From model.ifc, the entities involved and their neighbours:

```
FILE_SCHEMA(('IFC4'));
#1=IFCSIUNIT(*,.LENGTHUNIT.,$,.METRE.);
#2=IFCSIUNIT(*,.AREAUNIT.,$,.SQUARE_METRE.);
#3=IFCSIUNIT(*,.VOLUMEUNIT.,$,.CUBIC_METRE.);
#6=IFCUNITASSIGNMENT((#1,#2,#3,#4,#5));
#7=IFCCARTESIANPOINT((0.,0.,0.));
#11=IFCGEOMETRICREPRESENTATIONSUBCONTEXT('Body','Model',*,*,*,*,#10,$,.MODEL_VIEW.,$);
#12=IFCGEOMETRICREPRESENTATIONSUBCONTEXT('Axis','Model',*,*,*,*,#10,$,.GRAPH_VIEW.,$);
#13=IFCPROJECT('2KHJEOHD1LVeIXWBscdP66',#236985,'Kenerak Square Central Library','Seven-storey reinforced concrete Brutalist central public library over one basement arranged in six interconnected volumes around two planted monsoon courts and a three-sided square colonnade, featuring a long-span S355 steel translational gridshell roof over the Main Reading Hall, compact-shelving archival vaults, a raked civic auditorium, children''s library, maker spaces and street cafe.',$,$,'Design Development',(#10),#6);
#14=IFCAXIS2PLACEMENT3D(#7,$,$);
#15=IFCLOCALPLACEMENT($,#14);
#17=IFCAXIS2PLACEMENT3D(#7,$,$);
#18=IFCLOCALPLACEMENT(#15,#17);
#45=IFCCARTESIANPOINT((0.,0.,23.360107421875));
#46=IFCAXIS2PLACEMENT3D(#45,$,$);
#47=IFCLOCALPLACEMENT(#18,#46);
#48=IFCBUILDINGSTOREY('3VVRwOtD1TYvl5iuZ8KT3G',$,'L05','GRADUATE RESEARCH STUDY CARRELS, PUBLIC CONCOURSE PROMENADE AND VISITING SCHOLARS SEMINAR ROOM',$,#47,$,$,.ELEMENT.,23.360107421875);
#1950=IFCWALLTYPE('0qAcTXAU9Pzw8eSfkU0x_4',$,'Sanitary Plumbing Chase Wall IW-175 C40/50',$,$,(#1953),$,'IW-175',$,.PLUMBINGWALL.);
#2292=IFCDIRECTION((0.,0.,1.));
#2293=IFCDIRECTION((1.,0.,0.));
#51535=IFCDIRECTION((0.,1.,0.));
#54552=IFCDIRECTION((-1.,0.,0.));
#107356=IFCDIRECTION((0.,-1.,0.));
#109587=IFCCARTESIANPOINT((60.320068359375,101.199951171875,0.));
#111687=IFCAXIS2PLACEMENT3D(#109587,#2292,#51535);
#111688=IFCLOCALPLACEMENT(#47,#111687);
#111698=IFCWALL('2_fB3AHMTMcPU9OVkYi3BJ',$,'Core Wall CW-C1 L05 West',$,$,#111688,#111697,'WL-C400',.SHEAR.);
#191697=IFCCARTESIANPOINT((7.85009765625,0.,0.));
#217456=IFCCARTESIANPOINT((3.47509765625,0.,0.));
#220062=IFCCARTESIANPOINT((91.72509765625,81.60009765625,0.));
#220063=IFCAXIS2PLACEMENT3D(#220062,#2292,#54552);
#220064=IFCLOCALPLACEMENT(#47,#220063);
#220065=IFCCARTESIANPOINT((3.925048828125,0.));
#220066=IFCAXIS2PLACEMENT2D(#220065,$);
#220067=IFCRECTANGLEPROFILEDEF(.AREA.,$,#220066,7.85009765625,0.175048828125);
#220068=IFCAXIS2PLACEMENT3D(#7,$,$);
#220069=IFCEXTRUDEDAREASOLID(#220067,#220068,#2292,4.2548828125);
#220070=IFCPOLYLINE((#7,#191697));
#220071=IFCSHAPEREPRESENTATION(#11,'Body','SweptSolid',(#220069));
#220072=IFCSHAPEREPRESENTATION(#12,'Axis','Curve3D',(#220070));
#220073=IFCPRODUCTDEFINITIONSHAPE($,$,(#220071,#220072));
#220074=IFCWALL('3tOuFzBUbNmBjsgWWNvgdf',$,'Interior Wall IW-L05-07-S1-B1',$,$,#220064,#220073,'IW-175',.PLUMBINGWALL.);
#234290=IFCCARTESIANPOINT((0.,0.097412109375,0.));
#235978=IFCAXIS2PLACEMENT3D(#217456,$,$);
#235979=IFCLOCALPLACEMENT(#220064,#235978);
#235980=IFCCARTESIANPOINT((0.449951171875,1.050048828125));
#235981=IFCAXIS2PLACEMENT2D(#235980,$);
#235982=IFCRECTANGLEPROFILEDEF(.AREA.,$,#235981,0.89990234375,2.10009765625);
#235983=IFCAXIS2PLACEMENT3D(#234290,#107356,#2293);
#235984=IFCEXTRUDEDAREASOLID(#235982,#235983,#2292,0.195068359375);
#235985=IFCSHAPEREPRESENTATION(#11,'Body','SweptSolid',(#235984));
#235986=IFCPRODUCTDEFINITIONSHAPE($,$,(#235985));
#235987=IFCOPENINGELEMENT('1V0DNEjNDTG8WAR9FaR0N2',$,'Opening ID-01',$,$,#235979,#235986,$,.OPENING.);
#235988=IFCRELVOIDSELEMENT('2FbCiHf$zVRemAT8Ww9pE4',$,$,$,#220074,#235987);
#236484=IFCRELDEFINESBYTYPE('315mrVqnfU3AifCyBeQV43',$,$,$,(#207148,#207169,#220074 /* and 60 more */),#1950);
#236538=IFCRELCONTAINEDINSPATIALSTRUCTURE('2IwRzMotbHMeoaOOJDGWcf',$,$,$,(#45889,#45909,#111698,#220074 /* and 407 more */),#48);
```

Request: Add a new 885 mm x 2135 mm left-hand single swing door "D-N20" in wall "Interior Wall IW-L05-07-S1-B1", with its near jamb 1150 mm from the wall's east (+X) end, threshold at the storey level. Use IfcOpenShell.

```python
import numpy as np
import ifcopenshell
import ifcopenshell.api.feature
import ifcopenshell.api.geometry
import ifcopenshell.api.root
import ifcopenshell.api.spatial
import ifcopenshell.geom
import ifcopenshell.util.element
import ifcopenshell.util.placement
import ifcopenshell.util.representation
import ifcopenshell.util.shape
import ifcopenshell.util.unit

model = ifcopenshell.open("model.ifc")
unit_scale = ifcopenshell.util.unit.calculate_unit_scale(model)
settings = ifcopenshell.geom.settings()


def volume(element):
    """Net volume in cubic metres, openings subtracted."""
    shape = ifcopenshell.geom.create_shape(settings, element)
    return ifcopenshell.util.shape.get_volume(shape.geometry)


wall = model.by_guid("3tOuFzBUbNmBjsgWWNvgdf")
storey = ifcopenshell.util.element.get_container(wall, ifc_class="IfcBuildingStorey")
context = ifcopenshell.util.representation.get_context(model, "Model", "Body", "MODEL_VIEW")
before = volume(wall)

width, height, from_end, sill = 0.885, 2.135, 1.15, 0.0  # metres

# The wall runs along its own X axis, and the end named is its -X end.
wall_shape = ifcopenshell.geom.create_shape(settings, wall)
x, y, z = ifcopenshell.util.shape.get_vertices(wall_shape.geometry).T
start = x.min() + from_end
face, thickness = float(y.min()), float(y.max() - y.min())
wall_matrix = ifcopenshell.util.placement.get_local_placement(wall.ObjectPlacement)
level = ifcopenshell.util.placement.get_local_placement(storey.ObjectPlacement)[2, 3]


def in_wall(x, y):
    """Placement at x, y metres in the wall's axes, at sill height."""
    matrix = wall_matrix.copy()
    matrix[:, 3] = wall_matrix @ np.array([x / unit_scale, y / unit_scale, 0.0, 1.0])
    matrix[2, 3] = level + sill / unit_scale
    return matrix


# Opening: a box that overshoots both wall faces by 50 mm.
opening = ifcopenshell.api.root.create_entity(model, ifc_class="IfcOpeningElement", predefined_type="OPENING")
box = ifcopenshell.api.geometry.add_wall_representation(
    model, context=context, length=width, height=height, thickness=thickness + 0.1
)
ifcopenshell.api.geometry.assign_representation(model, product=opening, representation=box)
ifcopenshell.api.geometry.edit_object_placement(model, product=opening, matrix=in_wall(start, face - 0.05), is_si=False)
ifcopenshell.api.feature.add_feature(model, feature=opening, element=wall)

door = ifcopenshell.api.root.create_entity(model, ifc_class="IfcDoor", name="D-N20", predefined_type="DOOR")
door.OverallWidth, door.OverallHeight = width / unit_scale, height / unit_scale
door.OperationType = "SINGLE_SWING_LEFT"
body = ifcopenshell.api.geometry.add_door_representation(
    model,
    context=context,
    overall_width=door.OverallWidth,
    overall_height=door.OverallHeight,
    operation_type="SINGLE_SWING_LEFT",
    lining_properties={"LiningDepth": thickness / unit_scale, "ThresholdDepth": thickness / unit_scale},
)
ifcopenshell.api.geometry.assign_representation(model, product=door, representation=body)
ifcopenshell.api.spatial.assign_container(model, products=[door], relating_structure=storey)
ifcopenshell.api.feature.add_filling(model, opening=opening, element=door)

# The lining spans the wall, so the door starts at the wall face.
ifcopenshell.api.geometry.edit_object_placement(model, product=door, matrix=in_wall(start, face), is_si=False)

after = volume(wall)

print(f"wall volume {before:.3f} -> {after:.3f} m3")

model.write("model-out.ifc")
```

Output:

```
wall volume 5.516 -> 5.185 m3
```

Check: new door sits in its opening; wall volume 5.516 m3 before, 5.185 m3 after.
